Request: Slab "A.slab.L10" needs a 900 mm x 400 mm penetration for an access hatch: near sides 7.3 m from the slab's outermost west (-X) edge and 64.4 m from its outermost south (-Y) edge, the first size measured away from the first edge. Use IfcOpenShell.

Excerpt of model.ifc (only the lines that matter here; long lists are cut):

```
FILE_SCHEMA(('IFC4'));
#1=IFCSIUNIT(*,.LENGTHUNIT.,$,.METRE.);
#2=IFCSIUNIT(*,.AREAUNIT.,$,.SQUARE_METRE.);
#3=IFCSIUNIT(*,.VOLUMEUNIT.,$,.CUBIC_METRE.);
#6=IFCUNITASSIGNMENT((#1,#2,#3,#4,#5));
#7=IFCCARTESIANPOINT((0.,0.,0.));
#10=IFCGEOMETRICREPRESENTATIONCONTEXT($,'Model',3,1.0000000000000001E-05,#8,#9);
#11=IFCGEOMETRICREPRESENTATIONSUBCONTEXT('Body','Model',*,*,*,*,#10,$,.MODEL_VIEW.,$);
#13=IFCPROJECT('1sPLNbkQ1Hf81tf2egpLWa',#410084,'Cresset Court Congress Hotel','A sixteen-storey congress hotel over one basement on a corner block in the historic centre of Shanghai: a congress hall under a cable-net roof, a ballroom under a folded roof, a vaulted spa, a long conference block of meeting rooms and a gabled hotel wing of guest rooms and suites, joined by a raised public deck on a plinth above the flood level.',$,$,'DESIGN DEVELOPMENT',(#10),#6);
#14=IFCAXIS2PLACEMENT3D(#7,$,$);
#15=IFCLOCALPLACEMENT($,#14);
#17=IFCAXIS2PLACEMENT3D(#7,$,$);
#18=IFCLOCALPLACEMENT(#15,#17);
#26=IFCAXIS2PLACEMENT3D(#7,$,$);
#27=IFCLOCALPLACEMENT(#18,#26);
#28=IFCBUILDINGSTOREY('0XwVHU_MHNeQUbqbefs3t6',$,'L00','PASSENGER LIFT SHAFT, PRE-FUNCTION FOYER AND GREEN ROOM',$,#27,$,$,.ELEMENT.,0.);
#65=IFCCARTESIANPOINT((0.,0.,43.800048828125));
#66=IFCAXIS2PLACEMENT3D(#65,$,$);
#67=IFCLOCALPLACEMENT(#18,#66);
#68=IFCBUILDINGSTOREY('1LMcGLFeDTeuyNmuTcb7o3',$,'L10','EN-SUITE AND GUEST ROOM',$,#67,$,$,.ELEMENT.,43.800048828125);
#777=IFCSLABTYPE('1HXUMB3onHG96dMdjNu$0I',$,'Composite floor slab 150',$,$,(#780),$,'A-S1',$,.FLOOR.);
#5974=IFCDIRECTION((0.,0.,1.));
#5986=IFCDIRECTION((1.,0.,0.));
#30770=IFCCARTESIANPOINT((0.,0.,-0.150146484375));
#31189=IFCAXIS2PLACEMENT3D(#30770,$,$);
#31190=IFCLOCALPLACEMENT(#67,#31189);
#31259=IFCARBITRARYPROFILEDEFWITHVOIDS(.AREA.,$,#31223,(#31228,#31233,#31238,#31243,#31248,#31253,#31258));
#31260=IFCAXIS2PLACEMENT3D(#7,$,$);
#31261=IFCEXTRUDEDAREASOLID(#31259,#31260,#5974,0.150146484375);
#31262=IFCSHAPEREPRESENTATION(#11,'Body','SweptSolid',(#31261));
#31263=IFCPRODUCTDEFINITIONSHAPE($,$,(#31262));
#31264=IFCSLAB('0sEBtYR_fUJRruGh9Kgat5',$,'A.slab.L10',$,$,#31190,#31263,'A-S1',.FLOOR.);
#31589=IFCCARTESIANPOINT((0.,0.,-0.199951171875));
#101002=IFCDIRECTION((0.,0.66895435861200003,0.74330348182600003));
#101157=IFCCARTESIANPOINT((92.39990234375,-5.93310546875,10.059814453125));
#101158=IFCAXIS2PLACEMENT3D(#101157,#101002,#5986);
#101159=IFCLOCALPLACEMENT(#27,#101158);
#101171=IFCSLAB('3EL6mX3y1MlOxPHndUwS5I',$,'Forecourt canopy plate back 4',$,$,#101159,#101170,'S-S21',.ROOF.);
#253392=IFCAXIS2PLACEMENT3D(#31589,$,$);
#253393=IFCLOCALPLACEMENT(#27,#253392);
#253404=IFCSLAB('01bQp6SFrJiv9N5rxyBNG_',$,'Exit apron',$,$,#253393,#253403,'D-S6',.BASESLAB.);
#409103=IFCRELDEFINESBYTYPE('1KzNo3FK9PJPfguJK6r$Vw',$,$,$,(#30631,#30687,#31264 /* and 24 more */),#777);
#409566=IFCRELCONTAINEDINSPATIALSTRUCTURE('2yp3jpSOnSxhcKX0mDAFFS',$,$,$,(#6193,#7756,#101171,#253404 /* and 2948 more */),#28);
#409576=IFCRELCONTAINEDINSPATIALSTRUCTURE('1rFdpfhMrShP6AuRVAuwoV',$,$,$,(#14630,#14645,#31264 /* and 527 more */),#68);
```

```python
import numpy as np
import ifcopenshell
import ifcopenshell.api.feature
import ifcopenshell.api.geometry
import ifcopenshell.api.root
import ifcopenshell.geom
import ifcopenshell.util.placement
import ifcopenshell.util.representation
import ifcopenshell.util.shape
import ifcopenshell.util.unit

model = ifcopenshell.open("model.ifc")
unit_scale = ifcopenshell.util.unit.calculate_unit_scale(model)
settings = ifcopenshell.geom.settings()


def volume(element):
    """Net volume in cubic metres, openings subtracted."""
    shape = ifcopenshell.geom.create_shape(settings, element)
    return ifcopenshell.util.shape.get_volume(shape.geometry)


slab = model.by_guid("0sEBtYR_fUJRruGh9Kgat5")
before = volume(slab)

# Extent in the slab's own axes, in metres. The edges named are its -X and -Y sides.
slab_shape = ifcopenshell.geom.create_shape(settings, slab)
vertices = ifcopenshell.util.shape.get_vertices(slab_shape.geometry)
x_min, y_min, bottom = vertices.min(axis=0)
top = vertices[:, 2].max()

opening = ifcopenshell.api.root.create_entity(model, ifc_class="IfcOpeningElement", name="Access hatch opening", predefined_type="OPENING")
context = ifcopenshell.util.representation.get_context(model, "Model", "Body", "MODEL_VIEW")
width, depth = 0.9, 0.4
outline = [(0.0, 0.0), (width, 0.0), (width, depth), (0.0, depth), (0.0, 0.0)]
# Overshoot both faces by 50 mm so the cut is clean.
shape = ifcopenshell.api.geometry.add_slab_representation(
    model, context=context, depth=top - bottom + 0.1, polyline=outline
)
ifcopenshell.api.geometry.assign_representation(model, product=opening, representation=shape)

matrix = ifcopenshell.util.placement.get_local_placement(slab.ObjectPlacement)
matrix[:, 3] = matrix @ np.append(np.array([x_min + 7.3, y_min + 64.4, bottom - 0.05]) / unit_scale, 1.0)
ifcopenshell.api.geometry.edit_object_placement(model, product=opening, matrix=matrix, is_si=False)
ifcopenshell.api.feature.add_feature(model, feature=opening, element=slab)

after = volume(slab)

print(f"slab volume {before:.3f} -> {after:.3f} m3")

model.write("model-out.ifc")
```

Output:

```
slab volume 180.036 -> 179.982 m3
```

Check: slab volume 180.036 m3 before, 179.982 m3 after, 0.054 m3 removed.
